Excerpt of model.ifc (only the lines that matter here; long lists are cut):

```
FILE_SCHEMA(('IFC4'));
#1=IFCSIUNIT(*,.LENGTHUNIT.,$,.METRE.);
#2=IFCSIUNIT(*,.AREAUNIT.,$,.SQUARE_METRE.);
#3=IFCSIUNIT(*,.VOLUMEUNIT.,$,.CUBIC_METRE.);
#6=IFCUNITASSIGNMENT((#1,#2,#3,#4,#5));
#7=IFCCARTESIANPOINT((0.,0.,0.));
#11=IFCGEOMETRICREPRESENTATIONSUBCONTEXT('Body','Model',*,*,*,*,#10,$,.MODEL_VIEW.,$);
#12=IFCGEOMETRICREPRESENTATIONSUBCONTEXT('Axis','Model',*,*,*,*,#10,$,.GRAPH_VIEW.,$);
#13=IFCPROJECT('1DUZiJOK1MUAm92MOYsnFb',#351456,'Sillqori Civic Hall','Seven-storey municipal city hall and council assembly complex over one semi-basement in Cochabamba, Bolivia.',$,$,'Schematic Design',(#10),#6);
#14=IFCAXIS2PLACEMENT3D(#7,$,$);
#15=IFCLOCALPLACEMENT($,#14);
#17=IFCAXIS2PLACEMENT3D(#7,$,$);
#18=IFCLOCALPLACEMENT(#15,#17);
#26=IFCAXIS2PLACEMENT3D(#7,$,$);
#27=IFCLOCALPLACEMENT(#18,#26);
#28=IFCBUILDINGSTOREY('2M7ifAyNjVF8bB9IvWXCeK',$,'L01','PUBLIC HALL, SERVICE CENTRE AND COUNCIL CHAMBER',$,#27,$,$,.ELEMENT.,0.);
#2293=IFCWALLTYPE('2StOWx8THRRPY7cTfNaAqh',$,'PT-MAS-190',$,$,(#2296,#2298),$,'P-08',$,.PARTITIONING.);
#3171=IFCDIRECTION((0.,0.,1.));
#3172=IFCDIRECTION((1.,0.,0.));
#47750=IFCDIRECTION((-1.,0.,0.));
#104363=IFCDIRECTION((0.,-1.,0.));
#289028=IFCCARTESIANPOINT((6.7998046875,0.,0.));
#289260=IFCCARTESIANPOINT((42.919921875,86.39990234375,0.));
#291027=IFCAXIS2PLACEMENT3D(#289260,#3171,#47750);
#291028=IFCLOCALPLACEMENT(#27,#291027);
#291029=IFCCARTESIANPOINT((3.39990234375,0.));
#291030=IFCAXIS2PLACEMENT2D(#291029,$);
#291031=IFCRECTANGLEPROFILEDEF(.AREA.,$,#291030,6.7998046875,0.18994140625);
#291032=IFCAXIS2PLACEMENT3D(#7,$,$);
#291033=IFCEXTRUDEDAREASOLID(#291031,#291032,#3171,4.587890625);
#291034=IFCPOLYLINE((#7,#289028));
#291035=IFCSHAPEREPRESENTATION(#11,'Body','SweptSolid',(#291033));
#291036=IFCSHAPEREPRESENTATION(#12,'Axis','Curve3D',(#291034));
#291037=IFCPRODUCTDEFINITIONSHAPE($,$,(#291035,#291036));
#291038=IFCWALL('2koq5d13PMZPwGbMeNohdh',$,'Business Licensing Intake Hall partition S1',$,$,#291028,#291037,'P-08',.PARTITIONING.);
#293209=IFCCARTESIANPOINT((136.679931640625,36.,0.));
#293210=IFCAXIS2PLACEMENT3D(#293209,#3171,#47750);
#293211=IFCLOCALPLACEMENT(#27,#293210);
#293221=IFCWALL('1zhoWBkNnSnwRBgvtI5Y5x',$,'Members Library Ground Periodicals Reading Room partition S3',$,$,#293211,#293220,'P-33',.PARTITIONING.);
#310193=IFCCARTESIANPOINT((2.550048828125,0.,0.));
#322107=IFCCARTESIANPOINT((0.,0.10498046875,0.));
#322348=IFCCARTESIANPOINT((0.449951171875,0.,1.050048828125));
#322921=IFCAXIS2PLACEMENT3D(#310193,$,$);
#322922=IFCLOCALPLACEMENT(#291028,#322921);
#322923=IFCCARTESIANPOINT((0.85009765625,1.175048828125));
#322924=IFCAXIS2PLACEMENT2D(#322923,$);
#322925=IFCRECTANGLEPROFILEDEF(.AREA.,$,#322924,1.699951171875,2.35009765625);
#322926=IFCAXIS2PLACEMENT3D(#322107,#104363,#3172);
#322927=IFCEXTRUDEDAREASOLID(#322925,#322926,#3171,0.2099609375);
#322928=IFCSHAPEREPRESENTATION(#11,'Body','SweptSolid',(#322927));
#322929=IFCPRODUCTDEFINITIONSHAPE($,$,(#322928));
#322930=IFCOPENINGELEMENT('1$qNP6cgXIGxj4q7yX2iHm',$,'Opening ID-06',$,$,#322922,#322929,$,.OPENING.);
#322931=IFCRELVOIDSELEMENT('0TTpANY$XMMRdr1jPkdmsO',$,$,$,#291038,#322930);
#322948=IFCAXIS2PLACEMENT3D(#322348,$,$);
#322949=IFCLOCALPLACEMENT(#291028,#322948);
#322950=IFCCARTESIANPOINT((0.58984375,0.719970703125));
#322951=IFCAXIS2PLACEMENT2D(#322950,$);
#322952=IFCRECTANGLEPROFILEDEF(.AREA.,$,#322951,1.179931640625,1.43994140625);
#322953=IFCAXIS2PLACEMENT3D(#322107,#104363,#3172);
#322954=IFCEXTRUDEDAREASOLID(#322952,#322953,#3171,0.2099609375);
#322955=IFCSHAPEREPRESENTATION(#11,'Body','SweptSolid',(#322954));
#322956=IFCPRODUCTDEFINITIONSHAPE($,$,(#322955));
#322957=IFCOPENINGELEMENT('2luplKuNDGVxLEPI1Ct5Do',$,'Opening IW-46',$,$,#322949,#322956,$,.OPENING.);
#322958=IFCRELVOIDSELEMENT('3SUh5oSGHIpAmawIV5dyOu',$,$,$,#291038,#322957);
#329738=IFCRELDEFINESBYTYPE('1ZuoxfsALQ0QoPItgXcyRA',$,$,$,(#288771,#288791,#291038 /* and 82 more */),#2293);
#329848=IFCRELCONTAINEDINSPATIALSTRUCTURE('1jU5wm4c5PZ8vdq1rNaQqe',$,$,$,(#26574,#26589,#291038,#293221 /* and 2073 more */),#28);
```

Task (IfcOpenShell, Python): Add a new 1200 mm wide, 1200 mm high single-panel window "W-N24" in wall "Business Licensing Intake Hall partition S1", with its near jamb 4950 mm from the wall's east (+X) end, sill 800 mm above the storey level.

```python
import numpy as np
import ifcopenshell
import ifcopenshell.api.feature
import ifcopenshell.api.geometry
import ifcopenshell.api.root
import ifcopenshell.api.spatial
import ifcopenshell.geom
import ifcopenshell.util.element
import ifcopenshell.util.placement
import ifcopenshell.util.representation
import ifcopenshell.util.shape
import ifcopenshell.util.unit

model = ifcopenshell.open("model.ifc")
unit_scale = ifcopenshell.util.unit.calculate_unit_scale(model)
settings = ifcopenshell.geom.settings()


def volume(element):
    """Net volume in cubic metres, openings subtracted."""
    shape = ifcopenshell.geom.create_shape(settings, element)
    return ifcopenshell.util.shape.get_volume(shape.geometry)


wall = model.by_guid("2koq5d13PMZPwGbMeNohdh")
storey = ifcopenshell.util.element.get_container(wall, ifc_class="IfcBuildingStorey")
context = ifcopenshell.util.representation.get_context(model, "Model", "Body", "MODEL_VIEW")
before = volume(wall)

width, height, from_end, sill = 1.2, 1.2, 4.95, 0.8  # metres

# The wall runs along its own X axis, and the end named is its -X end.
wall_shape = ifcopenshell.geom.create_shape(settings, wall)
x, y, z = ifcopenshell.util.shape.get_vertices(wall_shape.geometry).T
start = x.min() + from_end
face, thickness = float(y.min()), float(y.max() - y.min())
wall_matrix = ifcopenshell.util.placement.get_local_placement(wall.ObjectPlacement)
level = ifcopenshell.util.placement.get_local_placement(storey.ObjectPlacement)[2, 3]


def in_wall(x, y):
    """Placement at x, y metres in the wall's axes, at sill height."""
    matrix = wall_matrix.copy()
    matrix[:, 3] = wall_matrix @ np.array([x / unit_scale, y / unit_scale, 0.0, 1.0])
    matrix[2, 3] = level + sill / unit_scale
    return matrix


# Opening: a box that overshoots both wall faces by 50 mm.
opening = ifcopenshell.api.root.create_entity(model, ifc_class="IfcOpeningElement", predefined_type="OPENING")
box = ifcopenshell.api.geometry.add_wall_representation(
    model, context=context, length=width, height=height, thickness=thickness + 0.1
)
ifcopenshell.api.geometry.assign_representation(model, product=opening, representation=box)
ifcopenshell.api.geometry.edit_object_placement(model, product=opening, matrix=in_wall(start, face - 0.05), is_si=False)
ifcopenshell.api.feature.add_feature(model, feature=opening, element=wall)

window = ifcopenshell.api.root.create_entity(model, ifc_class="IfcWindow", name="W-N24", predefined_type="WINDOW")
window.OverallWidth, window.OverallHeight = width / unit_scale, height / unit_scale
window.PartitioningType = "SINGLE_PANEL"
body = ifcopenshell.api.geometry.add_window_representation(
    model,
    context=context,
    overall_width=window.OverallWidth,
    overall_height=window.OverallHeight,
    partition_type="SINGLE_PANEL",
)
ifcopenshell.api.geometry.assign_representation(model, product=window, representation=body)
ifcopenshell.api.spatial.assign_container(model, products=[window], relating_structure=storey)
ifcopenshell.api.feature.add_filling(model, opening=opening, element=window)

# Centre the window in the wall's thickness.
ifcopenshell.api.geometry.edit_object_placement(model, product=window, matrix=in_wall(start, face), is_si=False)
window_shape = ifcopenshell.geom.create_shape(settings, window)
depth = ifcopenshell.util.shape.get_vertices(window_shape.geometry)[:, 1]
offset = face + thickness / 2 - (depth.min() + depth.max()) / 2
ifcopenshell.api.geometry.edit_object_placement(model, product=window, matrix=in_wall(start, offset), is_si=False)

after = volume(wall)

print(f"wall volume {before:.3f} -> {after:.3f} m3")

model.write("model_updated.ifc")
```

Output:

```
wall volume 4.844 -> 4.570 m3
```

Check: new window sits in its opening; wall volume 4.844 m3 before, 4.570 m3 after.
